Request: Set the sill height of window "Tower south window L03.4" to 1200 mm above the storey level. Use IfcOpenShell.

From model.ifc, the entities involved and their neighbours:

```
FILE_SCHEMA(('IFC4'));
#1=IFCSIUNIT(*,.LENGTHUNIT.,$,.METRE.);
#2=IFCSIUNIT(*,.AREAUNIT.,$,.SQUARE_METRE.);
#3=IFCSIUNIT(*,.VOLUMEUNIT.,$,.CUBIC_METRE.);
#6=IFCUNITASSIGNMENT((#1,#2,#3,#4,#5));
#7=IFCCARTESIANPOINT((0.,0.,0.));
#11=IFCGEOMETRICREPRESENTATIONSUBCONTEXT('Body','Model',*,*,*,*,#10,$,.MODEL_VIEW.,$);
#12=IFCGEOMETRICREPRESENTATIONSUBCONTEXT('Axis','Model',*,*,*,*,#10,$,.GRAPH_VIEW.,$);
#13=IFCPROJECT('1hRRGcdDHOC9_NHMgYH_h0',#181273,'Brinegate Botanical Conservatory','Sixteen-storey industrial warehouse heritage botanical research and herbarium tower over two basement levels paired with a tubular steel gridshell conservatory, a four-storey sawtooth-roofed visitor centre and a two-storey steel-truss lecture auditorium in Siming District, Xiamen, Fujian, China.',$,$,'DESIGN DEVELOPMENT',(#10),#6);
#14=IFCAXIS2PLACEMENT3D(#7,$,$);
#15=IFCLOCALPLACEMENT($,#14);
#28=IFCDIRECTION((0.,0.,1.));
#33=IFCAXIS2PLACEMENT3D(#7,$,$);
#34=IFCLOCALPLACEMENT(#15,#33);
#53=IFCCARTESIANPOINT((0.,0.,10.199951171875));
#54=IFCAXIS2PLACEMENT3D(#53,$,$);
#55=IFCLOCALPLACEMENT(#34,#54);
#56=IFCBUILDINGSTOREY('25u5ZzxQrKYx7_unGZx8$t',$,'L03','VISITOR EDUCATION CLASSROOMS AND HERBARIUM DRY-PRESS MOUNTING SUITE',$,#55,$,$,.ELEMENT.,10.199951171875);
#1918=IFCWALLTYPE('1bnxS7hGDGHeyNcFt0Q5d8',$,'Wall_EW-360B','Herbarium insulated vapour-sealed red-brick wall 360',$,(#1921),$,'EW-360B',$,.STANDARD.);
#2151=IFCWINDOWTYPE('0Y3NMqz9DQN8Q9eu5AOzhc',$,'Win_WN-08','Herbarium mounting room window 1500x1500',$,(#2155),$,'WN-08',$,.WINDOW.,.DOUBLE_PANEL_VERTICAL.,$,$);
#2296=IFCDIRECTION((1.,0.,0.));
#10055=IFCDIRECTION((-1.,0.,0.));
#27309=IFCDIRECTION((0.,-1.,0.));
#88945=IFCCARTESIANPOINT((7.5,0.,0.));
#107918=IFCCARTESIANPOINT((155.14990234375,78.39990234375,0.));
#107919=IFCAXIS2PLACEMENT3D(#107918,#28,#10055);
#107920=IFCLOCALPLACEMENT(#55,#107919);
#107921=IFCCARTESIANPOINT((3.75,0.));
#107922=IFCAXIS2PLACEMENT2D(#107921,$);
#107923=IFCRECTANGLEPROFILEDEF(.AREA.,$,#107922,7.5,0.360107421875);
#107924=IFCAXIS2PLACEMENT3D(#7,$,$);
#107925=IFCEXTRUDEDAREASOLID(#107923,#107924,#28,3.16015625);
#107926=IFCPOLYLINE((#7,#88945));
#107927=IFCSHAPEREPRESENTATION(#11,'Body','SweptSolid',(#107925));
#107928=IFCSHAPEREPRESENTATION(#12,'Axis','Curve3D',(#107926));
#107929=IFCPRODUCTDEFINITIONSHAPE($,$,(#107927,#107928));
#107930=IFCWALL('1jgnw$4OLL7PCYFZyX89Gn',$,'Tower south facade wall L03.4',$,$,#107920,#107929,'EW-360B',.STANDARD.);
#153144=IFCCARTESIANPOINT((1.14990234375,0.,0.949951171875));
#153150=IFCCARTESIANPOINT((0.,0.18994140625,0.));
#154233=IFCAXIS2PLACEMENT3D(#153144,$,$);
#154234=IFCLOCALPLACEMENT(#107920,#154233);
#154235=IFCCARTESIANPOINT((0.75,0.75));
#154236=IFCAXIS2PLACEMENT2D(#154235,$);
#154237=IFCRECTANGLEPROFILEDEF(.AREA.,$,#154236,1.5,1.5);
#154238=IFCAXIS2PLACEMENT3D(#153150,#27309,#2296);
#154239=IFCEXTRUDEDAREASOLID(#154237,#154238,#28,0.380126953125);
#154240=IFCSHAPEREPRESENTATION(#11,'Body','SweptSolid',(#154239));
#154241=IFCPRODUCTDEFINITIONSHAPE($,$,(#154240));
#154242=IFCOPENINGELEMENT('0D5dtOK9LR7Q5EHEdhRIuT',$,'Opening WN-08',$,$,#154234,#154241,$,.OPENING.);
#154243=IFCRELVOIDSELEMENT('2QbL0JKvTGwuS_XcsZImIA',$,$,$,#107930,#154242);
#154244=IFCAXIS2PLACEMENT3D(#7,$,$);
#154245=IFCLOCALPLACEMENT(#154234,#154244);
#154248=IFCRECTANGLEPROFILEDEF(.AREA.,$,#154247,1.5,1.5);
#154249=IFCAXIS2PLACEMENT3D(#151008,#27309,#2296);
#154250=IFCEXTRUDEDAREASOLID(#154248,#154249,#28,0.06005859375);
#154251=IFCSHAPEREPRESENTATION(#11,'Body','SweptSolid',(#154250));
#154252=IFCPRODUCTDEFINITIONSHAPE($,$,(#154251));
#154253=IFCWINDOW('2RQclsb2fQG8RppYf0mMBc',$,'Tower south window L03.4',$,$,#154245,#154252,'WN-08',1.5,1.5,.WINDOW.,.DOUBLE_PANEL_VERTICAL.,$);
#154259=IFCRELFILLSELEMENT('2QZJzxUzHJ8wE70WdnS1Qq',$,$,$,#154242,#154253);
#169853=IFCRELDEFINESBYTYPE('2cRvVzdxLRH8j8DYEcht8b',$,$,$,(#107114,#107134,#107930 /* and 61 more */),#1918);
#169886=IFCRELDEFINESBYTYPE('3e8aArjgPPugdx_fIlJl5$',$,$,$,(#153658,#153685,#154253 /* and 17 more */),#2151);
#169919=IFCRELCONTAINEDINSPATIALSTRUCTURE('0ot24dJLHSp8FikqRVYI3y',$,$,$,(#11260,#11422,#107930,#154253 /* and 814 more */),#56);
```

```python
import numpy as np
import ifcopenshell
import ifcopenshell.api.geometry
import ifcopenshell.geom
import ifcopenshell.util.element
import ifcopenshell.util.placement
import ifcopenshell.util.shape
import ifcopenshell.util.unit

model = ifcopenshell.open("model.ifc")
unit_scale = ifcopenshell.util.unit.calculate_unit_scale(model)

window = model.by_guid("2RQclsb2fQG8RppYf0mMBc")
opening = window.FillsVoids[0].RelatingOpeningElement
storey = ifcopenshell.util.element.get_container(window, ifc_class="IfcBuildingStorey")
level = ifcopenshell.util.placement.get_local_placement(storey.ObjectPlacement)[2, 3]

# The opening's origin need not be at the sill, so measure its lowest point.
shape = ifcopenshell.geom.create_shape(ifcopenshell.geom.settings(), opening)
bottom = ifcopenshell.util.shape.get_shape_bottom_elevation(shape, shape.geometry) / unit_scale
dz = level + 1.2 / unit_scale - bottom

shift = np.array([0.0, 0.0, dz])
# The window is placed relative to its opening, so it follows when the opening moves.
matrix = ifcopenshell.util.placement.get_local_placement(opening.ObjectPlacement)
matrix[:3, 3] += shift
ifcopenshell.api.geometry.edit_object_placement(
    model, product=opening, matrix=matrix, is_si=False, should_transform_children=True
)

print(f"moved by {dz * unit_scale:+.3f} m")

model.write("model_v2.ifc")
```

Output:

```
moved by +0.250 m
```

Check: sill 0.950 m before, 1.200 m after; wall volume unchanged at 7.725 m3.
